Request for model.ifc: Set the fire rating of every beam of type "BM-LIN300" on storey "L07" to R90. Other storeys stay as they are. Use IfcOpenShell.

First a look at what the model holds.

```python
import ifcopenshell
import ifcopenshell.util.element

model = ifcopenshell.open("model.ifc")
print(model.schema)
storey = next(s for s in model.by_type("IfcBuildingStorey") if s.Name == "L07")
beams = [e for e in ifcopenshell.util.element.get_decomposition(storey) if e.is_a("IfcBeam")]
seen = {}
for e in beams:
    element_type = ifcopenshell.util.element.get_type(e)
    key = (element_type.Name if element_type != e and element_type else None, ifcopenshell.util.element.get_pset(e, "Pset_BeamCommon", "FireRating"))
    seen[key] = seen.get(key, 0) + 1
for (name, value), count in sorted(seen.items(), key=str):
    print(count, "x", name, "|", value)
```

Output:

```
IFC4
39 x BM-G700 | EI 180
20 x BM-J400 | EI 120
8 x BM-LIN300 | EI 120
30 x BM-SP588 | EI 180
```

```python
import ifcopenshell
import ifcopenshell.api.pset
import ifcopenshell.util.element

model = ifcopenshell.open("model.ifc")

storey = next(s for s in model.by_type("IfcBuildingStorey") if s.Name == "L07")
beams = [e for e in ifcopenshell.util.element.get_decomposition(storey) if e.is_a("IfcBeam")]

count = 0
for e in beams:
    element_type = ifcopenshell.util.element.get_type(e)
    if element_type in (None, e) or element_type.Name != "BM-LIN300":
        continue
    found = ifcopenshell.util.element.get_pset(e, "Pset_BeamCommon", should_inherit=False)
    if found:
        pset = model.by_id(found["id"])
        if len(ifcopenshell.util.element.get_elements_by_pset(pset)) > 1:
            pset = ifcopenshell.api.pset.unshare_pset(model, products=[e], pset=pset)[0]
    else:
        pset = ifcopenshell.api.pset.add_pset(model, product=e, name="Pset_BeamCommon")
    ifcopenshell.api.pset.edit_pset(model, pset=pset, properties={"FireRating": "R90"})
    count += 1

print(count, "beams updated")

model.write("model_updated.ifc")
```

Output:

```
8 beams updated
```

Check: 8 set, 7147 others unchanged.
